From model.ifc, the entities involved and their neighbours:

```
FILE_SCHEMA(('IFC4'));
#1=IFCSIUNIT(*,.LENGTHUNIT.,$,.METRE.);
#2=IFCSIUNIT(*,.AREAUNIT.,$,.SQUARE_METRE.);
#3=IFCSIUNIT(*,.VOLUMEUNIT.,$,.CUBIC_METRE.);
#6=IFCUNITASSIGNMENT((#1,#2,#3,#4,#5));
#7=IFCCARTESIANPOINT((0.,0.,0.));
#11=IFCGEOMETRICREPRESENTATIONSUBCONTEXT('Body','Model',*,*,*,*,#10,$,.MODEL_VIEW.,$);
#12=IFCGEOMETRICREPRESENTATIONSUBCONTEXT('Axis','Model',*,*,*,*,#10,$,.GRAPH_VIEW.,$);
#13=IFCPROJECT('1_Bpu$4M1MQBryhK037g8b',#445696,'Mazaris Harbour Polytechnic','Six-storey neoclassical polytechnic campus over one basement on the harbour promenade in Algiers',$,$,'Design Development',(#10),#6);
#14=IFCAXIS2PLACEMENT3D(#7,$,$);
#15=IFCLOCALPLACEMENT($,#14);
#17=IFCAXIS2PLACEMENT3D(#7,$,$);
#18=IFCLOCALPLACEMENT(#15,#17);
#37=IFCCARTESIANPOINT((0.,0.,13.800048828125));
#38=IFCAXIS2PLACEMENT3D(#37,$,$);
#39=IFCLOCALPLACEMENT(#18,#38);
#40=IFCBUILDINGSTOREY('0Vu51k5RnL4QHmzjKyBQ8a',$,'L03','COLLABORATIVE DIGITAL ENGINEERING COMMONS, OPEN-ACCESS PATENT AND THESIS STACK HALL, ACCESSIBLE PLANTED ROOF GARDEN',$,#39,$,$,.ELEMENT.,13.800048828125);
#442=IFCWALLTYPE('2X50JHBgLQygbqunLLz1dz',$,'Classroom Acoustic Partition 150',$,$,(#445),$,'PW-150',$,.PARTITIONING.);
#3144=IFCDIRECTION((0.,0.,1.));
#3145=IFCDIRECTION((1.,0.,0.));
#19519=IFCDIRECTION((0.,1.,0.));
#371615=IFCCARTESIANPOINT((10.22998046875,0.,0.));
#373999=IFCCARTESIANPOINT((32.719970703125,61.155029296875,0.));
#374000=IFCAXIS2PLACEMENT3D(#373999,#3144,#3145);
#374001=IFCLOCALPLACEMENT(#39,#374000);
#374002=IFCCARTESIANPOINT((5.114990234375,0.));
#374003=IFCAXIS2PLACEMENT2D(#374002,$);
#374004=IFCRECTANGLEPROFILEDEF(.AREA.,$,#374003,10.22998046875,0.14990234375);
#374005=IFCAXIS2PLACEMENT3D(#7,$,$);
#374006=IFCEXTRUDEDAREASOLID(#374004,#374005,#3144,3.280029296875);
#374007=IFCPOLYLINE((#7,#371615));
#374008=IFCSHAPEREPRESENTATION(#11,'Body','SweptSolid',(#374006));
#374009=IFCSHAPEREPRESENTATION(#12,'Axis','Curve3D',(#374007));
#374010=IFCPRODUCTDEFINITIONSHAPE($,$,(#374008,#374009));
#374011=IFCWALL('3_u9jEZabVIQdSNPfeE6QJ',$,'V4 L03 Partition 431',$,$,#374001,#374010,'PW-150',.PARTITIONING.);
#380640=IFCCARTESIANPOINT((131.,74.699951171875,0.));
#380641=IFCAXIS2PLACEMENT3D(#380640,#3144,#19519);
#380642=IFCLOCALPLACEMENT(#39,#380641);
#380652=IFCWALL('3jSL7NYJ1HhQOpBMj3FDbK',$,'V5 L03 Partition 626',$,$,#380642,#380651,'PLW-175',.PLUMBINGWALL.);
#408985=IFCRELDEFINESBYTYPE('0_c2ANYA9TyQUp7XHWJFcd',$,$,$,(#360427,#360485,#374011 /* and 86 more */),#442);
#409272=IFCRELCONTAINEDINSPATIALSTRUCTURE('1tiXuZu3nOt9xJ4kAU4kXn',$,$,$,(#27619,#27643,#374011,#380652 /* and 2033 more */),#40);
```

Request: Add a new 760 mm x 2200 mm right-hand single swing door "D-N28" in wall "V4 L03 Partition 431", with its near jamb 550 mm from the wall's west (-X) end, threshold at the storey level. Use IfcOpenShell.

```python
import numpy as np
import ifcopenshell
import ifcopenshell.api.feature
import ifcopenshell.api.geometry
import ifcopenshell.api.root
import ifcopenshell.api.spatial
import ifcopenshell.geom
import ifcopenshell.util.element
import ifcopenshell.util.placement
import ifcopenshell.util.representation
import ifcopenshell.util.shape
import ifcopenshell.util.unit

model = ifcopenshell.open("model.ifc")
unit_scale = ifcopenshell.util.unit.calculate_unit_scale(model)
settings = ifcopenshell.geom.settings()


def volume(element):
    """Net volume in cubic metres, openings subtracted."""
    shape = ifcopenshell.geom.create_shape(settings, element)
    return ifcopenshell.util.shape.get_volume(shape.geometry)


wall = model.by_guid("3_u9jEZabVIQdSNPfeE6QJ")
storey = ifcopenshell.util.element.get_container(wall, ifc_class="IfcBuildingStorey")
context = ifcopenshell.util.representation.get_context(model, "Model", "Body", "MODEL_VIEW")
before = volume(wall)

width, height, from_end, sill = 0.76, 2.2, 0.55, 0.0  # metres

# The wall runs along its own X axis, and the end named is its -X end.
wall_shape = ifcopenshell.geom.create_shape(settings, wall)
x, y, z = ifcopenshell.util.shape.get_vertices(wall_shape.geometry).T
start = x.min() + from_end
face, thickness = float(y.min()), float(y.max() - y.min())
wall_matrix = ifcopenshell.util.placement.get_local_placement(wall.ObjectPlacement)
level = ifcopenshell.util.placement.get_local_placement(storey.ObjectPlacement)[2, 3]


def in_wall(x, y):
    """Placement at x, y metres in the wall's axes, at sill height."""
    matrix = wall_matrix.copy()
    matrix[:, 3] = wall_matrix @ np.array([x / unit_scale, y / unit_scale, 0.0, 1.0])
    matrix[2, 3] = level + sill / unit_scale
    return matrix


# Opening: a box that overshoots both wall faces by 50 mm.
opening = ifcopenshell.api.root.create_entity(model, ifc_class="IfcOpeningElement", predefined_type="OPENING")
box = ifcopenshell.api.geometry.add_wall_representation(
    model, context=context, length=width, height=height, thickness=thickness + 0.1
)
ifcopenshell.api.geometry.assign_representation(model, product=opening, representation=box)
ifcopenshell.api.geometry.edit_object_placement(model, product=opening, matrix=in_wall(start, face - 0.05), is_si=False)
ifcopenshell.api.feature.add_feature(model, feature=opening, element=wall)

door = ifcopenshell.api.root.create_entity(model, ifc_class="IfcDoor", name="D-N28", predefined_type="DOOR")
door.OverallWidth, door.OverallHeight = width / unit_scale, height / unit_scale
door.OperationType = "SINGLE_SWING_RIGHT"
body = ifcopenshell.api.geometry.add_door_representation(
    model,
    context=context,
    overall_width=door.OverallWidth,
    overall_height=door.OverallHeight,
    operation_type="SINGLE_SWING_RIGHT",
    lining_properties={"LiningDepth": thickness / unit_scale, "ThresholdDepth": thickness / unit_scale},
)
ifcopenshell.api.geometry.assign_representation(model, product=door, representation=body)
ifcopenshell.api.spatial.assign_container(model, products=[door], relating_structure=storey)
ifcopenshell.api.feature.add_filling(model, opening=opening, element=door)

# The lining spans the wall, so the door starts at the wall face.
ifcopenshell.api.geometry.edit_object_placement(model, product=door, matrix=in_wall(start, face), is_si=False)

after = volume(wall)

print(f"wall volume {before:.3f} -> {after:.3f} m3")

model.write("model_updated.ifc")
```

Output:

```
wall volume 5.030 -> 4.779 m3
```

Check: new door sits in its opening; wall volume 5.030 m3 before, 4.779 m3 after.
